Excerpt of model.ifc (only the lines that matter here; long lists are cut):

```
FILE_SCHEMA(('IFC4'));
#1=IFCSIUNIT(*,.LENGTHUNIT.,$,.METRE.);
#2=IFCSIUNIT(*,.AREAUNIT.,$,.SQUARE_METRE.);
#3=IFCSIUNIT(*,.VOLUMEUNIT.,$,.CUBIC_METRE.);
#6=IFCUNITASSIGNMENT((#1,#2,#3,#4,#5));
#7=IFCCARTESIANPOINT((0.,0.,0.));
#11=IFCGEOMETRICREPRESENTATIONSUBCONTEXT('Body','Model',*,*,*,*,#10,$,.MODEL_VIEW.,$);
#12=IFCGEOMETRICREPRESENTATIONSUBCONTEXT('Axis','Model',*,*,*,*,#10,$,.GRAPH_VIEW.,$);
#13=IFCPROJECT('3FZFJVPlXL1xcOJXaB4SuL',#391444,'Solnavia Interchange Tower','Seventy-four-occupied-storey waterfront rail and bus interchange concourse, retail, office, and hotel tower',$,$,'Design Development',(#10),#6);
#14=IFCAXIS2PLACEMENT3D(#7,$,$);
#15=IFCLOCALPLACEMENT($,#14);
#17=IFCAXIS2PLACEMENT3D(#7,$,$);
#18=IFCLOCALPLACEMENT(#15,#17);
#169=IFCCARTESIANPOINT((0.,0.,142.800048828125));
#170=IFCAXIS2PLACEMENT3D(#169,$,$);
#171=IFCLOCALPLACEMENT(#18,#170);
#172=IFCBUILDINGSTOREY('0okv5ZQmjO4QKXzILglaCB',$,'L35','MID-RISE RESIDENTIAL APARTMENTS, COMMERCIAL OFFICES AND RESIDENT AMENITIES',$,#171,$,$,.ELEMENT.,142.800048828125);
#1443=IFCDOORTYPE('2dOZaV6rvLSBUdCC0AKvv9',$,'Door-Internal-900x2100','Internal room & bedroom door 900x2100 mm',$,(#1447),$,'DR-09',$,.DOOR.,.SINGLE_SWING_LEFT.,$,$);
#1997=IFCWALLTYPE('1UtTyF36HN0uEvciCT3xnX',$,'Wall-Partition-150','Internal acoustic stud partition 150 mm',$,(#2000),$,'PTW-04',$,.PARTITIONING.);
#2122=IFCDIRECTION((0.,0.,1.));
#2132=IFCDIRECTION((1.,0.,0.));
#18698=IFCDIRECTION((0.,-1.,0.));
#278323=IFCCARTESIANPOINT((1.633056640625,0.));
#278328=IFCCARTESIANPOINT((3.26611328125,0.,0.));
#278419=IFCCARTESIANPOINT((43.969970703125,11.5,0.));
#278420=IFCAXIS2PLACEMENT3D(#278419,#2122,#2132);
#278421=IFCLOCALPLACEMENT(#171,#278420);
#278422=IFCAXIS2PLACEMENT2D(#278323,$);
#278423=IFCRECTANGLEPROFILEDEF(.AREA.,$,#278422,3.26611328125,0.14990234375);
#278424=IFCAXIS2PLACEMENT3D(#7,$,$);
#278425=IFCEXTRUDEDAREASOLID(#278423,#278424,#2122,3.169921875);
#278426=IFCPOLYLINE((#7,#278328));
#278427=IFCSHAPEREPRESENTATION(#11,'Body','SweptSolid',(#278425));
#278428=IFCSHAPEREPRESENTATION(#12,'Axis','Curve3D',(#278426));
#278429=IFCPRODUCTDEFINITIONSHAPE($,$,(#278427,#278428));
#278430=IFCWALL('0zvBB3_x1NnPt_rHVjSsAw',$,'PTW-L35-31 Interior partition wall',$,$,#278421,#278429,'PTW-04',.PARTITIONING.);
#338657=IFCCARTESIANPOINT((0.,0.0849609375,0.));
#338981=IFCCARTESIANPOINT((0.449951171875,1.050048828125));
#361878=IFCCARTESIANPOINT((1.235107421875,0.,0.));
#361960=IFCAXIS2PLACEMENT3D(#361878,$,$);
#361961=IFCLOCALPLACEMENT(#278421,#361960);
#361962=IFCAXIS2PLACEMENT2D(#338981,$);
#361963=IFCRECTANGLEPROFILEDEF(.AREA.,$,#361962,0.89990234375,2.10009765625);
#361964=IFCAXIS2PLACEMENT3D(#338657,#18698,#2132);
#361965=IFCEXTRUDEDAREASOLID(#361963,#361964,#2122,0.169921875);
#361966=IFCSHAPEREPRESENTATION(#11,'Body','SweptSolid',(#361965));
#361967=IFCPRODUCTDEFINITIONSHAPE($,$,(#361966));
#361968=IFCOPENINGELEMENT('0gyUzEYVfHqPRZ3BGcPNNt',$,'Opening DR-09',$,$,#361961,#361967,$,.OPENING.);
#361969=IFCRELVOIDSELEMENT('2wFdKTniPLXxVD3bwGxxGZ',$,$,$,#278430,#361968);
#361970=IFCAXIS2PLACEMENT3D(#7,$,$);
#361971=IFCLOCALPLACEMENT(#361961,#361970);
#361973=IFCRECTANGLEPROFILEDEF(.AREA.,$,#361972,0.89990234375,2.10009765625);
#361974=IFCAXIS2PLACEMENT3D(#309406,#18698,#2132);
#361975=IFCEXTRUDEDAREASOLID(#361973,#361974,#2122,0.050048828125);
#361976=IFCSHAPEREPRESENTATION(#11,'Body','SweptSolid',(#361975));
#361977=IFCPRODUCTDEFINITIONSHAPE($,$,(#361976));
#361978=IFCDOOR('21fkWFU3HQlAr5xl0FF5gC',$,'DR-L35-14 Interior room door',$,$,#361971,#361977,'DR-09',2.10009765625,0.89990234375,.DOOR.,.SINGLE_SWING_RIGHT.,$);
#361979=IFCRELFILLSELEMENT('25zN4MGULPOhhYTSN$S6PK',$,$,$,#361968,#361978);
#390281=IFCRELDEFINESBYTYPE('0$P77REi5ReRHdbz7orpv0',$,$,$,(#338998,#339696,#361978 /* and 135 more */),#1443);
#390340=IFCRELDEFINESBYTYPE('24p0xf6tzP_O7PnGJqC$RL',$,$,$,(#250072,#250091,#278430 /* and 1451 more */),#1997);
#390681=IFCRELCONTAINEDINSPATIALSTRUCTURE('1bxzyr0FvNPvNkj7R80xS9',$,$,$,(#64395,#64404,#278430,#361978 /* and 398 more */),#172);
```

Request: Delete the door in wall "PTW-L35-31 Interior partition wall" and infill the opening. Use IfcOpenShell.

```python
import ifcopenshell
import ifcopenshell.api.feature
import ifcopenshell.api.root
import ifcopenshell.geom
import ifcopenshell.util.shape

model = ifcopenshell.open("model.ifc")
settings = ifcopenshell.geom.settings()


def volume(element):
    """Net volume in cubic metres, openings subtracted."""
    shape = ifcopenshell.geom.create_shape(settings, element)
    return ifcopenshell.util.shape.get_volume(shape.geometry)


door = model.by_guid("21fkWFU3HQlAr5xl0FF5gC")
opening = door.FillsVoids[0].RelatingOpeningElement
wall = opening.VoidsElements[0].RelatingBuildingElement
before = volume(wall)

ifcopenshell.api.root.remove_product(model, product=door)
ifcopenshell.api.feature.remove_feature(model, feature=opening)

after = volume(wall)

print(f"wall volume {before:.3f} -> {after:.3f} m3")

model.write("model_edited.ifc")
```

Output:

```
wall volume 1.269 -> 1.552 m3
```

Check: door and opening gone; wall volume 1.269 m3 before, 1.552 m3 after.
